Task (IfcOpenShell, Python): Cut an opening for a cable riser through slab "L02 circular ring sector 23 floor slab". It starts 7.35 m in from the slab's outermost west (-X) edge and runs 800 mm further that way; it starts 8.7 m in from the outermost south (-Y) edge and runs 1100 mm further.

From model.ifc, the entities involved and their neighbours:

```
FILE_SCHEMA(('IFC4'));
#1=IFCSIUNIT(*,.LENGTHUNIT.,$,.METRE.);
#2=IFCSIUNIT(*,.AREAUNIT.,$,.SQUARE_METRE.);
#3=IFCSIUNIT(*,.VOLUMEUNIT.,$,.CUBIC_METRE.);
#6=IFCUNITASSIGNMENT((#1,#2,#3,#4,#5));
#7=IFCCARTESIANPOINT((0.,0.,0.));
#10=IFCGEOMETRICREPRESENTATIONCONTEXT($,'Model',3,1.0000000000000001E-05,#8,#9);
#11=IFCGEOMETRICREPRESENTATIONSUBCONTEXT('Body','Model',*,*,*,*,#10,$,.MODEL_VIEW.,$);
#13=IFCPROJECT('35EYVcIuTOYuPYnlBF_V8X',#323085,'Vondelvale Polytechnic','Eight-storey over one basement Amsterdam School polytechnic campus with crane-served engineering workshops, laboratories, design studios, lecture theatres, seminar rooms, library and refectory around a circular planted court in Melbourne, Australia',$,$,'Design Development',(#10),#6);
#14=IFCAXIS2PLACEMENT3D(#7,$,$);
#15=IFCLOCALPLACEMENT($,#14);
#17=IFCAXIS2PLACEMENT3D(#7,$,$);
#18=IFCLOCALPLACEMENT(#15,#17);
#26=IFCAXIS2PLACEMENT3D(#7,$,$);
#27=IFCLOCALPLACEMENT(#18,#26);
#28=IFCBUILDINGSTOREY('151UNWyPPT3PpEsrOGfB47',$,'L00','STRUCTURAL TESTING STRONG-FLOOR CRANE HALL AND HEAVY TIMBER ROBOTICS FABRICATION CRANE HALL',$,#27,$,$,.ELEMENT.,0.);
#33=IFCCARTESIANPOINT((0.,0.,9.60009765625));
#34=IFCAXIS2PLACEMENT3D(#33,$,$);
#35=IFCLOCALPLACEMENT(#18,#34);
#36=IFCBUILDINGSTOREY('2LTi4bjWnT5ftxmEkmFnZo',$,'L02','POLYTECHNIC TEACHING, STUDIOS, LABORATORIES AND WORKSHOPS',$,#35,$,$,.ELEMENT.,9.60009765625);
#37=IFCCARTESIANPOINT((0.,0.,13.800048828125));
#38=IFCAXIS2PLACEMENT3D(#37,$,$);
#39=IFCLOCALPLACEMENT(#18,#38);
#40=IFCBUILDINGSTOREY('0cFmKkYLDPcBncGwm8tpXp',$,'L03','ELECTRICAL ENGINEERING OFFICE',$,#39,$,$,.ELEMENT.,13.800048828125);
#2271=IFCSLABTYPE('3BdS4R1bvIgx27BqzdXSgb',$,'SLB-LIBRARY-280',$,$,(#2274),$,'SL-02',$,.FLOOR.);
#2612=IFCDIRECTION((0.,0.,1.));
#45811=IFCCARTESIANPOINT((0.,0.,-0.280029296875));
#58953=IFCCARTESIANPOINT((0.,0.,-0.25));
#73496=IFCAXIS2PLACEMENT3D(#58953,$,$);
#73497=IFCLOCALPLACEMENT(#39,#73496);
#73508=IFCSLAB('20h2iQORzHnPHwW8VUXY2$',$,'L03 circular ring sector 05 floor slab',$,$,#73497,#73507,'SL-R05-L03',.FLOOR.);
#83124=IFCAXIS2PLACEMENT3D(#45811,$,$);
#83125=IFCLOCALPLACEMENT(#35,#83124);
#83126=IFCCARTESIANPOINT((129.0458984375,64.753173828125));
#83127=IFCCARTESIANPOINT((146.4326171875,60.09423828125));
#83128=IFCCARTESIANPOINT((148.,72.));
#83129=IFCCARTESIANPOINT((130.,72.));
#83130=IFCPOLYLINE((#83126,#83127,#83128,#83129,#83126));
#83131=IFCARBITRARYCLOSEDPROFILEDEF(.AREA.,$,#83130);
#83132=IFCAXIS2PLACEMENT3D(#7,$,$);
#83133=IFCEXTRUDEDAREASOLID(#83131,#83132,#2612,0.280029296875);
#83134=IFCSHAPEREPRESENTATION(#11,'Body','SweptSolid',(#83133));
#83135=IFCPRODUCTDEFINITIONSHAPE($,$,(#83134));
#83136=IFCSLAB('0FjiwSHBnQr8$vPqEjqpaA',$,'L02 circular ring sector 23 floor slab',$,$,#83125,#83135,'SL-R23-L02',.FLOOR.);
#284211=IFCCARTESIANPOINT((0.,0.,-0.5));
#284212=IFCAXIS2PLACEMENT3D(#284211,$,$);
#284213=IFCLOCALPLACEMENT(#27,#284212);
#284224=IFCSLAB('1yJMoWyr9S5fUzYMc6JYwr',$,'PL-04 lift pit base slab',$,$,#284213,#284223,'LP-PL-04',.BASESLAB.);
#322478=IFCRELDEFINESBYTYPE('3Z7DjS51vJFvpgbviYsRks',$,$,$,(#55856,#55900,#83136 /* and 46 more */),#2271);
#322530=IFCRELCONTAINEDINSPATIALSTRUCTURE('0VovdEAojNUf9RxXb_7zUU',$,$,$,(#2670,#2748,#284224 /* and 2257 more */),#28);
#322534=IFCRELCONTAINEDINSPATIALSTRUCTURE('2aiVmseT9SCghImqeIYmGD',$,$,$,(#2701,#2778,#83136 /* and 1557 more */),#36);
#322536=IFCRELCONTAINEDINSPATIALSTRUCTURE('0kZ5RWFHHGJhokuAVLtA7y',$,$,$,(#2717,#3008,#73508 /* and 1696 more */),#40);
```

```python
import numpy as np
import ifcopenshell
import ifcopenshell.api.feature
import ifcopenshell.api.geometry
import ifcopenshell.api.root
import ifcopenshell.geom
import ifcopenshell.util.placement
import ifcopenshell.util.representation
import ifcopenshell.util.shape
import ifcopenshell.util.unit

model = ifcopenshell.open("model.ifc")
unit_scale = ifcopenshell.util.unit.calculate_unit_scale(model)
settings = ifcopenshell.geom.settings()


def volume(element):
    """Net volume in cubic metres, openings subtracted."""
    shape = ifcopenshell.geom.create_shape(settings, element)
    return ifcopenshell.util.shape.get_volume(shape.geometry)


slab = model.by_id(83136)
before = volume(slab)

# Extent in the slab's own axes, in metres. The edges named are its -X and -Y sides.
slab_shape = ifcopenshell.geom.create_shape(settings, slab)
vertices = ifcopenshell.util.shape.get_vertices(slab_shape.geometry)
x_min, y_min, bottom = vertices.min(axis=0)
top = vertices[:, 2].max()

opening = ifcopenshell.api.root.create_entity(model, ifc_class="IfcOpeningElement", name="Cable riser opening", predefined_type="OPENING")
context = ifcopenshell.util.representation.get_context(model, "Model", "Body", "MODEL_VIEW")
width, depth = 0.8, 1.1
outline = [(0.0, 0.0), (width, 0.0), (width, depth), (0.0, depth), (0.0, 0.0)]
# Overshoot both faces by 50 mm so the cut is clean.
shape = ifcopenshell.api.geometry.add_slab_representation(
    model, context=context, depth=top - bottom + 0.1, polyline=outline
)
ifcopenshell.api.geometry.assign_representation(model, product=opening, representation=shape)

matrix = ifcopenshell.util.placement.get_local_placement(slab.ObjectPlacement)
matrix[:, 3] = matrix @ np.append(np.array([x_min + 7.35, y_min + 8.7, bottom - 0.05]) / unit_scale, 1.0)
ifcopenshell.api.geometry.edit_object_placement(model, product=opening, matrix=matrix, is_si=False)
ifcopenshell.api.feature.add_feature(model, feature=opening, element=slab)

after = volume(slab)

print(f"slab volume {before:.3f} -> {after:.3f} m3")

model.write("model-out.ifc")
```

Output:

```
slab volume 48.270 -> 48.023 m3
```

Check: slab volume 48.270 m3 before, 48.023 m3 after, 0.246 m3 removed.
